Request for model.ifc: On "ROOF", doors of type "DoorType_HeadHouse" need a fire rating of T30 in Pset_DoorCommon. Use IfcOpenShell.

First a look at what the model holds.

```python
import ifcopenshell
import ifcopenshell.util.element

model = ifcopenshell.open("model.ifc")
print(model.schema)
storey = next(s for s in model.by_type("IfcBuildingStorey") if s.Name == "ROOF")
doors = [e for e in ifcopenshell.util.element.get_decomposition(storey) if e.is_a("IfcDoor")]
seen = {}
for e in doors:
    element_type = ifcopenshell.util.element.get_type(e)
    key = (element_type.Name if element_type != e and element_type else None, ifcopenshell.util.element.get_pset(e, "Pset_DoorCommon", "FireRating"))
    seen[key] = seen.get(key, 0) + 1
for (name, value), count in sorted(seen.items(), key=str):
    print(count, "x", name, "|", value)
```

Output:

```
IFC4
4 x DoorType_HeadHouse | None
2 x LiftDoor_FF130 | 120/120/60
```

```python
import ifcopenshell
import ifcopenshell.api.pset
import ifcopenshell.util.element

model = ifcopenshell.open("model.ifc")

storey = next(s for s in model.by_type("IfcBuildingStorey") if s.Name == "ROOF")
doors = [e for e in ifcopenshell.util.element.get_decomposition(storey) if e.is_a("IfcDoor")]

count = 0
for e in doors:
    element_type = ifcopenshell.util.element.get_type(e)
    if element_type in (None, e) or element_type.Name != "DoorType_HeadHouse":
        continue
    # add_pset returns the element's existing set when there is one.
    pset = ifcopenshell.api.pset.add_pset(model, product=e, name="Pset_DoorCommon")
    ifcopenshell.api.pset.edit_pset(model, pset=pset, properties={"FireRating": "T30"})
    count += 1

print(count, "doors updated")

model.write("model-out.ifc")
```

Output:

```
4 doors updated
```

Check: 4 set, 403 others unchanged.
